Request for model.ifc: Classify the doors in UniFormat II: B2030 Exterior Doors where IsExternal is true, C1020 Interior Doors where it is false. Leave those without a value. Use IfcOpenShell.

First a look at what the model holds.

```python
import ifcopenshell
import ifcopenshell.util.element

model = ifcopenshell.open("model.ifc")
print(model.schema)
print("classifications:", [c.Name for c in model.by_type("IfcClassification")])
values = [ifcopenshell.util.element.get_pset(e, "Pset_DoorCommon", "IsExternal") for e in model.by_type("IfcDoor")]
for value in (True, False, None):
    print("IsExternal", value, values.count(value))
```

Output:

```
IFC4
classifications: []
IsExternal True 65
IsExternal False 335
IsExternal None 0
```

```python
import ifcopenshell
import ifcopenshell.api.classification
import ifcopenshell.util.element

model = ifcopenshell.open("model.ifc")

system = ifcopenshell.api.classification.add_classification(model, classification="UniFormat II")

doors = model.by_type("IfcDoor")
external = {e: ifcopenshell.util.element.get_pset(e, "Pset_DoorCommon", "IsExternal") for e in doors}
for flag, code, name in ((True, "B2030", "Exterior Doors"), (False, "C1020", "Interior Doors")):
    products = [e for e in doors if external[e] is flag]
    ifcopenshell.api.classification.add_reference(
        model, products=products, classification=system, identification=code, name=name
    )
    print(code, len(products))

model.write("model_rev.ifc")
```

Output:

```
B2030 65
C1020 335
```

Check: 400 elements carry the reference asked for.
